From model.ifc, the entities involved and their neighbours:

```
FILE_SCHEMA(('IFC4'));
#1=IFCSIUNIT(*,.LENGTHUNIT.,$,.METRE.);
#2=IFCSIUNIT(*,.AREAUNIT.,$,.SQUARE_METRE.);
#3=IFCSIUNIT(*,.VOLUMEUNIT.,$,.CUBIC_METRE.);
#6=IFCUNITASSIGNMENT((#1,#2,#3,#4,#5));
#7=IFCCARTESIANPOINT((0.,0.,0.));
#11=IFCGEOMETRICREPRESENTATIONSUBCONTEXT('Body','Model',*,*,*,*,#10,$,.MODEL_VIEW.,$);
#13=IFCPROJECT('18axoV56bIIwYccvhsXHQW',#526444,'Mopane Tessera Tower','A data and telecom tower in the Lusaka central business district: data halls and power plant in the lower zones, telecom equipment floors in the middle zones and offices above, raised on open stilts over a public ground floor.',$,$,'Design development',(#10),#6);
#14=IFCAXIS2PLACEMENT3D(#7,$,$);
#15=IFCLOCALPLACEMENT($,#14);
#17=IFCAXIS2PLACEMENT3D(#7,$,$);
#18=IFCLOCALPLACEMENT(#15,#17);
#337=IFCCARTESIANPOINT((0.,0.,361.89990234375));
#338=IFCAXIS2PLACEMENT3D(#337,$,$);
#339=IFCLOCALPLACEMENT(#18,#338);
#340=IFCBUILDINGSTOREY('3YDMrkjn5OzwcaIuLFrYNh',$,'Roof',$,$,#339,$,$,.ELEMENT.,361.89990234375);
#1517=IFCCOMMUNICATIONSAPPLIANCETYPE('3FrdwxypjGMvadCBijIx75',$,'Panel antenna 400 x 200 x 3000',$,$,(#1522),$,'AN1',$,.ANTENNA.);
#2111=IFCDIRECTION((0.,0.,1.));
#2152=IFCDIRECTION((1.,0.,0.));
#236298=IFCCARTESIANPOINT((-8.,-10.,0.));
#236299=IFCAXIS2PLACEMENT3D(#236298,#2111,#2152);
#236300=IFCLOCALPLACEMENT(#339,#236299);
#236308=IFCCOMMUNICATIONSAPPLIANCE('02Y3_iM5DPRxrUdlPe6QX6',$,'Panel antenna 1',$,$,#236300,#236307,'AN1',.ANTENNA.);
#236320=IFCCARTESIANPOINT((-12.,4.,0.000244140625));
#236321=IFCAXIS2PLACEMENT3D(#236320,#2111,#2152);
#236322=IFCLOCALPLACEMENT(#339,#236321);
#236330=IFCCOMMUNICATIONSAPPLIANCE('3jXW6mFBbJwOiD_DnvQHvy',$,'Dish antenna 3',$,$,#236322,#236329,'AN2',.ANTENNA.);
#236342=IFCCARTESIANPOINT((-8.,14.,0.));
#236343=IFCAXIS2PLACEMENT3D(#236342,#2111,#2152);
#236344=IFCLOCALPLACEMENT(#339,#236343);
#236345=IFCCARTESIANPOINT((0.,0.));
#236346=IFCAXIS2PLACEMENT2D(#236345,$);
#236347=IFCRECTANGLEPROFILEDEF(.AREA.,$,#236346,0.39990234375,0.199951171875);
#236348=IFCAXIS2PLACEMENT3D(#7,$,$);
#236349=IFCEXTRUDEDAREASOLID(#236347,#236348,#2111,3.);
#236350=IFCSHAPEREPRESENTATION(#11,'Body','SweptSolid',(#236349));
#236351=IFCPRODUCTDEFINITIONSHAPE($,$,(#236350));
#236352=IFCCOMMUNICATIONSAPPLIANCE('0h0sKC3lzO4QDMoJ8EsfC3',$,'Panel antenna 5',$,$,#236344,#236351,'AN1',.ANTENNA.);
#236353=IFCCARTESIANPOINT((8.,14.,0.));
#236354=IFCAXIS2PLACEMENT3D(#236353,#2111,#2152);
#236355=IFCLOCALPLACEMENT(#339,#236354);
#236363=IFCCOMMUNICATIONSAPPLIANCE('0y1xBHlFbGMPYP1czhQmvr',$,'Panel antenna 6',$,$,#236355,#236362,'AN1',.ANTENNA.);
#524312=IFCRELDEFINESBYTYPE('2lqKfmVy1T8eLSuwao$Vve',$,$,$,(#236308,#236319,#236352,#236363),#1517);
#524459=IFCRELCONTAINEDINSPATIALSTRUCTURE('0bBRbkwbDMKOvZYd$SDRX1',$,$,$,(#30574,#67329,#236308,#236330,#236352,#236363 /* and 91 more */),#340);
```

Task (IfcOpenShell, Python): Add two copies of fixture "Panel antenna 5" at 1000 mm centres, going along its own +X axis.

```python
import ifcopenshell
import ifcopenshell.api.geometry
import ifcopenshell.api.root
import ifcopenshell.util.element
import ifcopenshell.util.placement

model = ifcopenshell.open("model.ifc")

source = model.by_guid("0h0sKC3lzO4QDMoJ8EsfC3")
base = ifcopenshell.util.placement.get_local_placement(source.ObjectPlacement)
step = base[:3, 0] * 1.0

for i in range(1, 3):
    copy = ifcopenshell.api.root.copy_class(model, product=source)
    copy.Representation = ifcopenshell.util.element.copy_deep(
        model, source.Representation, exclude=["IfcGeometricRepresentationContext", "IfcRepresentationMap"]
    )
    copy.Tag = None
    matrix = base.copy()
    matrix[:3, 3] += i * step
    print("added at", matrix[:3, 3].round(3) + 0.0)
    ifcopenshell.api.geometry.edit_object_placement(model, product=copy, matrix=matrix, is_si=False)

model.write("model-out.ifc")
```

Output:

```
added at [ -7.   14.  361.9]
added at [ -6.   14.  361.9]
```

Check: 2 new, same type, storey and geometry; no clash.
